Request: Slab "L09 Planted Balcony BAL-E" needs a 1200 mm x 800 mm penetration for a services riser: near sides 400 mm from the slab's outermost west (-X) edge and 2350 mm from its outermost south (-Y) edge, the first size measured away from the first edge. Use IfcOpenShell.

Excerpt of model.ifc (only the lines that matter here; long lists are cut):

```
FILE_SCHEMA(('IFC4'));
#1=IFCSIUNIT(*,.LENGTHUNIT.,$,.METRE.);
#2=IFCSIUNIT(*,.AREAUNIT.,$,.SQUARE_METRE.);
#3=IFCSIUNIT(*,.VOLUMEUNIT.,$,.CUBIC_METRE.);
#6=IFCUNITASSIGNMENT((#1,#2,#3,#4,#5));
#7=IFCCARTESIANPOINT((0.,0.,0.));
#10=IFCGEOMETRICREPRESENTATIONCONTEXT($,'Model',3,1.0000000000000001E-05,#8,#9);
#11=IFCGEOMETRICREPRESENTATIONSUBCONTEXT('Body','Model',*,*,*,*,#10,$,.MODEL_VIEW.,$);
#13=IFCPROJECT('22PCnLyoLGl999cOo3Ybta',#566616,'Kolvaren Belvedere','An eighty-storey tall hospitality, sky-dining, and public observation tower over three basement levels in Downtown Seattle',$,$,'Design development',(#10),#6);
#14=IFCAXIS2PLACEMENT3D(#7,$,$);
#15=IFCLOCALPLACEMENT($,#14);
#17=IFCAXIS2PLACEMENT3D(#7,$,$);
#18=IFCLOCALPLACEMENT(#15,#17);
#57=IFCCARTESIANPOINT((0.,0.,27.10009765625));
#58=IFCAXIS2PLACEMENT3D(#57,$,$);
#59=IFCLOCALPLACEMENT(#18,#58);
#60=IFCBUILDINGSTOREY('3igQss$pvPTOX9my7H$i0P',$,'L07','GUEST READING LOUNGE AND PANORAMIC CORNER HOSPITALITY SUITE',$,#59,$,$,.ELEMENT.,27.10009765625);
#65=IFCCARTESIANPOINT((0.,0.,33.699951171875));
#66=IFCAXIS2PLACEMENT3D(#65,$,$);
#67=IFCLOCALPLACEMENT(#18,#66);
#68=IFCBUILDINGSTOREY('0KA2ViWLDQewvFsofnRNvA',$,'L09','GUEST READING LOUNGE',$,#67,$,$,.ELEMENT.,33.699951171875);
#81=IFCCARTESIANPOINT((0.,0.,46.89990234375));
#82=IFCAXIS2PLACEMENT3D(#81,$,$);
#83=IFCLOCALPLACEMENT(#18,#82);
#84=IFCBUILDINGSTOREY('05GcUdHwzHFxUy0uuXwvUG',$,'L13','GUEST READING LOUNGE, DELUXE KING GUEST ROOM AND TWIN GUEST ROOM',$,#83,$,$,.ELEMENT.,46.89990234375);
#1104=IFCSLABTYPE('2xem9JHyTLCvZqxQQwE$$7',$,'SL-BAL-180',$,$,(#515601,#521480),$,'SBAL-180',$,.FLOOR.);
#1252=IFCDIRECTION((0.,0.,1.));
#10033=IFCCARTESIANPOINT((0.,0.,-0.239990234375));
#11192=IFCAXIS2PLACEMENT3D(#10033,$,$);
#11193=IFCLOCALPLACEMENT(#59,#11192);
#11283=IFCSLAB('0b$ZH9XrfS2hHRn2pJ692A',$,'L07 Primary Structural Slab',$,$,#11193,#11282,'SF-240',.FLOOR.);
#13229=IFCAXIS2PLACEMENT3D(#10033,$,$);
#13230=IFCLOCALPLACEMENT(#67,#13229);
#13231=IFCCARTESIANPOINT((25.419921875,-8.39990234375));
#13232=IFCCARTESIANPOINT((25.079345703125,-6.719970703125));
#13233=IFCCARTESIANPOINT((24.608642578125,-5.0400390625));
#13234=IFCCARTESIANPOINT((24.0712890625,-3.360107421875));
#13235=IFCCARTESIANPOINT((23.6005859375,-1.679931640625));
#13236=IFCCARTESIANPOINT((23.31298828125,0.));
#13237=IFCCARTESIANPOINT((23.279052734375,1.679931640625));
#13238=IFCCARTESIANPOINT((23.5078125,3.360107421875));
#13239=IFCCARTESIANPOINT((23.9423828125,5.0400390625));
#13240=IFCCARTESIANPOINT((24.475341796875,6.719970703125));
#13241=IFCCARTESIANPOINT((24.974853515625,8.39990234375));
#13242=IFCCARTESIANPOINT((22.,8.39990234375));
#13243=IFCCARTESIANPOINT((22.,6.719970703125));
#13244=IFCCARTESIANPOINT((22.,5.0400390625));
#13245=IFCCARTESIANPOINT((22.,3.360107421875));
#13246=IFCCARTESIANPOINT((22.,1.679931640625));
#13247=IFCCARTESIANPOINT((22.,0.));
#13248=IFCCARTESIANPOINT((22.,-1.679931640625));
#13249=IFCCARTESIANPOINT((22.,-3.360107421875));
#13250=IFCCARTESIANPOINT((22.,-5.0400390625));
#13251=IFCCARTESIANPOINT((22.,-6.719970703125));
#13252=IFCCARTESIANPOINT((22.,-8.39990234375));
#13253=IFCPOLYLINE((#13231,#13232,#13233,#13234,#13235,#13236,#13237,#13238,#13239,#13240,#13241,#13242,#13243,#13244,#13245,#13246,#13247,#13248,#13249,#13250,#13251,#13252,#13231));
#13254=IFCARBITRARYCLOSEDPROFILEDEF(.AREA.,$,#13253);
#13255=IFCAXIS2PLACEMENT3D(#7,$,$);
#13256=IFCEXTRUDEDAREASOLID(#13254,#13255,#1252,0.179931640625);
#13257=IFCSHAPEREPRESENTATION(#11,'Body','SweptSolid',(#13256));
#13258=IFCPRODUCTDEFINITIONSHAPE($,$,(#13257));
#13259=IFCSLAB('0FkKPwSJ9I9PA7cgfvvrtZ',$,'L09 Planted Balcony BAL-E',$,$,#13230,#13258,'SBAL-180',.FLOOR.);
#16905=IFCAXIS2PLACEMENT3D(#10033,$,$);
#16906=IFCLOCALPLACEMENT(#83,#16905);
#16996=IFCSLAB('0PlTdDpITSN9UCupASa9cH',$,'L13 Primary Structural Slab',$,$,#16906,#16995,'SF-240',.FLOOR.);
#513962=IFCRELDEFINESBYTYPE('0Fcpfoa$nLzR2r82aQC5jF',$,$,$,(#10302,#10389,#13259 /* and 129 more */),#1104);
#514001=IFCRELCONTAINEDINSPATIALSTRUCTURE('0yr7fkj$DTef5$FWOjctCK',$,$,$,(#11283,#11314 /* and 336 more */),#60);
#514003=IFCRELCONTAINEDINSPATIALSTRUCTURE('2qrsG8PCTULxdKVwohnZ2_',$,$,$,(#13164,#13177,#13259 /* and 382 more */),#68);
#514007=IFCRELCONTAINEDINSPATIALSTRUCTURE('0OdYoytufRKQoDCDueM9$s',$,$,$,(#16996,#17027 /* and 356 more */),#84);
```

```python
import numpy as np
import ifcopenshell
import ifcopenshell.api.feature
import ifcopenshell.api.geometry
import ifcopenshell.api.root
import ifcopenshell.geom
import ifcopenshell.util.placement
import ifcopenshell.util.representation
import ifcopenshell.util.shape
import ifcopenshell.util.unit

model = ifcopenshell.open("model.ifc")
unit_scale = ifcopenshell.util.unit.calculate_unit_scale(model)
settings = ifcopenshell.geom.settings()


def volume(element):
    """Net volume in cubic metres, openings subtracted."""
    shape = ifcopenshell.geom.create_shape(settings, element)
    return ifcopenshell.util.shape.get_volume(shape.geometry)


slab = model.by_guid("0FkKPwSJ9I9PA7cgfvvrtZ")
before = volume(slab)

# Extent in the slab's own axes, in metres. The edges named are its -X and -Y sides.
slab_shape = ifcopenshell.geom.create_shape(settings, slab)
vertices = ifcopenshell.util.shape.get_vertices(slab_shape.geometry)
x_min, y_min, bottom = vertices.min(axis=0)
top = vertices[:, 2].max()

opening = ifcopenshell.api.root.create_entity(model, ifc_class="IfcOpeningElement", name="Services riser opening", predefined_type="OPENING")
context = ifcopenshell.util.representation.get_context(model, "Model", "Body", "MODEL_VIEW")
width, depth = 1.2, 0.8
outline = [(0.0, 0.0), (width, 0.0), (width, depth), (0.0, depth), (0.0, 0.0)]
# Overshoot both faces by 50 mm so the cut is clean.
shape = ifcopenshell.api.geometry.add_slab_representation(
    model, context=context, depth=top - bottom + 0.1, polyline=outline
)
ifcopenshell.api.geometry.assign_representation(model, product=opening, representation=shape)

matrix = ifcopenshell.util.placement.get_local_placement(slab.ObjectPlacement)
matrix[:, 3] = matrix @ np.append(np.array([x_min + 0.4, y_min + 2.35, bottom - 0.05]) / unit_scale, 1.0)
ifcopenshell.api.geometry.edit_object_placement(model, product=opening, matrix=matrix, is_si=False)
ifcopenshell.api.feature.add_feature(model, feature=opening, element=slab)

after = volume(slab)

print(f"slab volume {before:.3f} -> {after:.3f} m3")

model.write("model_v2.ifc")
```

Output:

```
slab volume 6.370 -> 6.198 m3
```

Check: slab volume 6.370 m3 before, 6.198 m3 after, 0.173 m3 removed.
